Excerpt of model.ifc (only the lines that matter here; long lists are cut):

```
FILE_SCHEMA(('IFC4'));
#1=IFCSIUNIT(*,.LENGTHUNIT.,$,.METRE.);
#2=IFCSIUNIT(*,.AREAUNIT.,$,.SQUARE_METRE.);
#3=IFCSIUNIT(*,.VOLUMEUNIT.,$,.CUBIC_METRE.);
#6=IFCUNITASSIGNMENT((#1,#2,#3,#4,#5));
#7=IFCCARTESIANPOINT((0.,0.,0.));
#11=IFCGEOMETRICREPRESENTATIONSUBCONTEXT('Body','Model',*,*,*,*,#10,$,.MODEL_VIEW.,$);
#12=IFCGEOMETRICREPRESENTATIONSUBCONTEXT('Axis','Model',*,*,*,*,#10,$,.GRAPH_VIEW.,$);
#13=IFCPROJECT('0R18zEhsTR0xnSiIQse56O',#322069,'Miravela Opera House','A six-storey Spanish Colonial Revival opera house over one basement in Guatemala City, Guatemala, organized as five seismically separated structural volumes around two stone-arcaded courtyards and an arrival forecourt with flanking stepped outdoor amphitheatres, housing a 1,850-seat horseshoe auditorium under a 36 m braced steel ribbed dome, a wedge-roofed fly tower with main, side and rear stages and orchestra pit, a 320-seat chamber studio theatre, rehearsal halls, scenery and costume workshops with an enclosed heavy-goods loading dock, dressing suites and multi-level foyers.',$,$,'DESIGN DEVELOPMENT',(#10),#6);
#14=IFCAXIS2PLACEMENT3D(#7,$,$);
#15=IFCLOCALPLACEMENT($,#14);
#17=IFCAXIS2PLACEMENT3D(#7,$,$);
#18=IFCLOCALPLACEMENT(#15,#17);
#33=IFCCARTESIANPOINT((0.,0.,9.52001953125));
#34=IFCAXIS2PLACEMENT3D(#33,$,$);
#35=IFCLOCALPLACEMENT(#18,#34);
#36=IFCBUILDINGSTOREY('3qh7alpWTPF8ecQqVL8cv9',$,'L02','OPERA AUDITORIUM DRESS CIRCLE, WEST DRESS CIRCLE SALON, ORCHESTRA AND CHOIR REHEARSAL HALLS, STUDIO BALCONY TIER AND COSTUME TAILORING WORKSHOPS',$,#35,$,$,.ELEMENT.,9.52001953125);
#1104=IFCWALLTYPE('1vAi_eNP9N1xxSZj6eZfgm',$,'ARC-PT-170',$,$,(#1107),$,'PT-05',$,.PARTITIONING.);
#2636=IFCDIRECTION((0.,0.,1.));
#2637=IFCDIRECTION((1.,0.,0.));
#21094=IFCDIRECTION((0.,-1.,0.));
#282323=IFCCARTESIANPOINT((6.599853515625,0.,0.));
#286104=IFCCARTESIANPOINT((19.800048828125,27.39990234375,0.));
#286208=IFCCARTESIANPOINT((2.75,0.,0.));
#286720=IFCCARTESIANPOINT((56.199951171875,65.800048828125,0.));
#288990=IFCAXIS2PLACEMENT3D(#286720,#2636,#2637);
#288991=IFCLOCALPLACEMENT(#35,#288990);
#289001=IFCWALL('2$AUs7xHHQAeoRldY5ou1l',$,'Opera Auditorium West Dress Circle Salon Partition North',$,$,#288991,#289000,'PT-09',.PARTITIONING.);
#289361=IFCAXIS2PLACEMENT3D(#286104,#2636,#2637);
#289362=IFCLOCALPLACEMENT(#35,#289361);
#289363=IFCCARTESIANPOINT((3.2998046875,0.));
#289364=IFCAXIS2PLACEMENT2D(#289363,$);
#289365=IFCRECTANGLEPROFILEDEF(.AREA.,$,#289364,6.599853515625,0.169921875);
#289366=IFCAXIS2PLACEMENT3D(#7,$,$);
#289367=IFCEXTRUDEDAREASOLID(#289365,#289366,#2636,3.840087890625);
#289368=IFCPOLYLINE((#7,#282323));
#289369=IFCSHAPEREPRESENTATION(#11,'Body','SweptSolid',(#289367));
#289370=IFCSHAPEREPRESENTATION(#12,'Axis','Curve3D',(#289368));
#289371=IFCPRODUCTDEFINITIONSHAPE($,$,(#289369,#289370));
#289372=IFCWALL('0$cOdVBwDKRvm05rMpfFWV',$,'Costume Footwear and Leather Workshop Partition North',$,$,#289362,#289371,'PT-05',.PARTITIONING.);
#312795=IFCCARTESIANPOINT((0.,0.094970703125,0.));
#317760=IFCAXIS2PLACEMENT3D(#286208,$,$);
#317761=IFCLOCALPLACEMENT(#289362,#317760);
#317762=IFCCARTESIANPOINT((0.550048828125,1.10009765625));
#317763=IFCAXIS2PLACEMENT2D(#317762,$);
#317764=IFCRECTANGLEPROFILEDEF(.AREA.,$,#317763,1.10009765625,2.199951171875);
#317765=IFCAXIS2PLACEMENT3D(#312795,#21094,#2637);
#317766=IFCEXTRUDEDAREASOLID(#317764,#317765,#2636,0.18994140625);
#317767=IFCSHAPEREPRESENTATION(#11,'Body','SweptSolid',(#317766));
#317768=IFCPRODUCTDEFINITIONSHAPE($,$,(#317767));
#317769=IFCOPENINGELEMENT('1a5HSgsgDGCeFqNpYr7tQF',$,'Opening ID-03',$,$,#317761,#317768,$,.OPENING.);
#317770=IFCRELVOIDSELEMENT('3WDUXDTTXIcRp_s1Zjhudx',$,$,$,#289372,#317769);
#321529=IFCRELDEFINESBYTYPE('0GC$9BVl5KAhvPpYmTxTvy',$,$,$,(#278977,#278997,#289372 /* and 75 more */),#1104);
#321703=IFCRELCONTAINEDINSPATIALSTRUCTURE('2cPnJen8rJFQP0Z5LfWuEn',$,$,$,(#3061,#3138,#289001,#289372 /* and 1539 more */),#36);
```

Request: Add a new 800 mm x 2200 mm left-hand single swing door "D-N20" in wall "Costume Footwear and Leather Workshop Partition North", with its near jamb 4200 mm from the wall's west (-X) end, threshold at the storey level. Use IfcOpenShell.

```python
import numpy as np
import ifcopenshell
import ifcopenshell.api.feature
import ifcopenshell.api.geometry
import ifcopenshell.api.root
import ifcopenshell.api.spatial
import ifcopenshell.geom
import ifcopenshell.util.element
import ifcopenshell.util.placement
import ifcopenshell.util.representation
import ifcopenshell.util.shape
import ifcopenshell.util.unit

model = ifcopenshell.open("model.ifc")
unit_scale = ifcopenshell.util.unit.calculate_unit_scale(model)
settings = ifcopenshell.geom.settings()


def volume(element):
    """Net volume in cubic metres, openings subtracted."""
    shape = ifcopenshell.geom.create_shape(settings, element)
    return ifcopenshell.util.shape.get_volume(shape.geometry)


wall = model.by_guid("0$cOdVBwDKRvm05rMpfFWV")
storey = ifcopenshell.util.element.get_container(wall, ifc_class="IfcBuildingStorey")
context = ifcopenshell.util.representation.get_context(model, "Model", "Body", "MODEL_VIEW")
before = volume(wall)

width, height, from_end, sill = 0.8, 2.2, 4.2, 0.0  # metres

# The wall runs along its own X axis, and the end named is its -X end.
wall_shape = ifcopenshell.geom.create_shape(settings, wall)
x, y, z = ifcopenshell.util.shape.get_vertices(wall_shape.geometry).T
start = x.min() + from_end
face, thickness = float(y.min()), float(y.max() - y.min())
wall_matrix = ifcopenshell.util.placement.get_local_placement(wall.ObjectPlacement)
level = ifcopenshell.util.placement.get_local_placement(storey.ObjectPlacement)[2, 3]


def in_wall(x, y):
    """Placement at x, y metres in the wall's axes, at sill height."""
    matrix = wall_matrix.copy()
    matrix[:, 3] = wall_matrix @ np.array([x / unit_scale, y / unit_scale, 0.0, 1.0])
    matrix[2, 3] = level + sill / unit_scale
    return matrix


# Opening: a box that overshoots both wall faces by 50 mm.
opening = ifcopenshell.api.root.create_entity(model, ifc_class="IfcOpeningElement", predefined_type="OPENING")
box = ifcopenshell.api.geometry.add_wall_representation(
    model, context=context, length=width, height=height, thickness=thickness + 0.1
)
ifcopenshell.api.geometry.assign_representation(model, product=opening, representation=box)
ifcopenshell.api.geometry.edit_object_placement(model, product=opening, matrix=in_wall(start, face - 0.05), is_si=False)
ifcopenshell.api.feature.add_feature(model, feature=opening, element=wall)

door = ifcopenshell.api.root.create_entity(model, ifc_class="IfcDoor", name="D-N20", predefined_type="DOOR")
door.OverallWidth, door.OverallHeight = width / unit_scale, height / unit_scale
door.OperationType = "SINGLE_SWING_LEFT"
body = ifcopenshell.api.geometry.add_door_representation(
    model,
    context=context,
    overall_width=door.OverallWidth,
    overall_height=door.OverallHeight,
    operation_type="SINGLE_SWING_LEFT",
    lining_properties={"LiningDepth": thickness / unit_scale, "ThresholdDepth": thickness / unit_scale},
)
ifcopenshell.api.geometry.assign_representation(model, product=door, representation=body)
ifcopenshell.api.spatial.assign_container(model, products=[door], relating_structure=storey)
ifcopenshell.api.feature.add_filling(model, opening=opening, element=door)

# The lining spans the wall, so the door starts at the wall face.
ifcopenshell.api.geometry.edit_object_placement(model, product=door, matrix=in_wall(start, face), is_si=False)

after = volume(wall)

print(f"wall volume {before:.3f} -> {after:.3f} m3")

model.write("model_edited.ifc")
```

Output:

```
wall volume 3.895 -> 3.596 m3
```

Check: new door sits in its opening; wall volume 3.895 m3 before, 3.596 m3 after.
